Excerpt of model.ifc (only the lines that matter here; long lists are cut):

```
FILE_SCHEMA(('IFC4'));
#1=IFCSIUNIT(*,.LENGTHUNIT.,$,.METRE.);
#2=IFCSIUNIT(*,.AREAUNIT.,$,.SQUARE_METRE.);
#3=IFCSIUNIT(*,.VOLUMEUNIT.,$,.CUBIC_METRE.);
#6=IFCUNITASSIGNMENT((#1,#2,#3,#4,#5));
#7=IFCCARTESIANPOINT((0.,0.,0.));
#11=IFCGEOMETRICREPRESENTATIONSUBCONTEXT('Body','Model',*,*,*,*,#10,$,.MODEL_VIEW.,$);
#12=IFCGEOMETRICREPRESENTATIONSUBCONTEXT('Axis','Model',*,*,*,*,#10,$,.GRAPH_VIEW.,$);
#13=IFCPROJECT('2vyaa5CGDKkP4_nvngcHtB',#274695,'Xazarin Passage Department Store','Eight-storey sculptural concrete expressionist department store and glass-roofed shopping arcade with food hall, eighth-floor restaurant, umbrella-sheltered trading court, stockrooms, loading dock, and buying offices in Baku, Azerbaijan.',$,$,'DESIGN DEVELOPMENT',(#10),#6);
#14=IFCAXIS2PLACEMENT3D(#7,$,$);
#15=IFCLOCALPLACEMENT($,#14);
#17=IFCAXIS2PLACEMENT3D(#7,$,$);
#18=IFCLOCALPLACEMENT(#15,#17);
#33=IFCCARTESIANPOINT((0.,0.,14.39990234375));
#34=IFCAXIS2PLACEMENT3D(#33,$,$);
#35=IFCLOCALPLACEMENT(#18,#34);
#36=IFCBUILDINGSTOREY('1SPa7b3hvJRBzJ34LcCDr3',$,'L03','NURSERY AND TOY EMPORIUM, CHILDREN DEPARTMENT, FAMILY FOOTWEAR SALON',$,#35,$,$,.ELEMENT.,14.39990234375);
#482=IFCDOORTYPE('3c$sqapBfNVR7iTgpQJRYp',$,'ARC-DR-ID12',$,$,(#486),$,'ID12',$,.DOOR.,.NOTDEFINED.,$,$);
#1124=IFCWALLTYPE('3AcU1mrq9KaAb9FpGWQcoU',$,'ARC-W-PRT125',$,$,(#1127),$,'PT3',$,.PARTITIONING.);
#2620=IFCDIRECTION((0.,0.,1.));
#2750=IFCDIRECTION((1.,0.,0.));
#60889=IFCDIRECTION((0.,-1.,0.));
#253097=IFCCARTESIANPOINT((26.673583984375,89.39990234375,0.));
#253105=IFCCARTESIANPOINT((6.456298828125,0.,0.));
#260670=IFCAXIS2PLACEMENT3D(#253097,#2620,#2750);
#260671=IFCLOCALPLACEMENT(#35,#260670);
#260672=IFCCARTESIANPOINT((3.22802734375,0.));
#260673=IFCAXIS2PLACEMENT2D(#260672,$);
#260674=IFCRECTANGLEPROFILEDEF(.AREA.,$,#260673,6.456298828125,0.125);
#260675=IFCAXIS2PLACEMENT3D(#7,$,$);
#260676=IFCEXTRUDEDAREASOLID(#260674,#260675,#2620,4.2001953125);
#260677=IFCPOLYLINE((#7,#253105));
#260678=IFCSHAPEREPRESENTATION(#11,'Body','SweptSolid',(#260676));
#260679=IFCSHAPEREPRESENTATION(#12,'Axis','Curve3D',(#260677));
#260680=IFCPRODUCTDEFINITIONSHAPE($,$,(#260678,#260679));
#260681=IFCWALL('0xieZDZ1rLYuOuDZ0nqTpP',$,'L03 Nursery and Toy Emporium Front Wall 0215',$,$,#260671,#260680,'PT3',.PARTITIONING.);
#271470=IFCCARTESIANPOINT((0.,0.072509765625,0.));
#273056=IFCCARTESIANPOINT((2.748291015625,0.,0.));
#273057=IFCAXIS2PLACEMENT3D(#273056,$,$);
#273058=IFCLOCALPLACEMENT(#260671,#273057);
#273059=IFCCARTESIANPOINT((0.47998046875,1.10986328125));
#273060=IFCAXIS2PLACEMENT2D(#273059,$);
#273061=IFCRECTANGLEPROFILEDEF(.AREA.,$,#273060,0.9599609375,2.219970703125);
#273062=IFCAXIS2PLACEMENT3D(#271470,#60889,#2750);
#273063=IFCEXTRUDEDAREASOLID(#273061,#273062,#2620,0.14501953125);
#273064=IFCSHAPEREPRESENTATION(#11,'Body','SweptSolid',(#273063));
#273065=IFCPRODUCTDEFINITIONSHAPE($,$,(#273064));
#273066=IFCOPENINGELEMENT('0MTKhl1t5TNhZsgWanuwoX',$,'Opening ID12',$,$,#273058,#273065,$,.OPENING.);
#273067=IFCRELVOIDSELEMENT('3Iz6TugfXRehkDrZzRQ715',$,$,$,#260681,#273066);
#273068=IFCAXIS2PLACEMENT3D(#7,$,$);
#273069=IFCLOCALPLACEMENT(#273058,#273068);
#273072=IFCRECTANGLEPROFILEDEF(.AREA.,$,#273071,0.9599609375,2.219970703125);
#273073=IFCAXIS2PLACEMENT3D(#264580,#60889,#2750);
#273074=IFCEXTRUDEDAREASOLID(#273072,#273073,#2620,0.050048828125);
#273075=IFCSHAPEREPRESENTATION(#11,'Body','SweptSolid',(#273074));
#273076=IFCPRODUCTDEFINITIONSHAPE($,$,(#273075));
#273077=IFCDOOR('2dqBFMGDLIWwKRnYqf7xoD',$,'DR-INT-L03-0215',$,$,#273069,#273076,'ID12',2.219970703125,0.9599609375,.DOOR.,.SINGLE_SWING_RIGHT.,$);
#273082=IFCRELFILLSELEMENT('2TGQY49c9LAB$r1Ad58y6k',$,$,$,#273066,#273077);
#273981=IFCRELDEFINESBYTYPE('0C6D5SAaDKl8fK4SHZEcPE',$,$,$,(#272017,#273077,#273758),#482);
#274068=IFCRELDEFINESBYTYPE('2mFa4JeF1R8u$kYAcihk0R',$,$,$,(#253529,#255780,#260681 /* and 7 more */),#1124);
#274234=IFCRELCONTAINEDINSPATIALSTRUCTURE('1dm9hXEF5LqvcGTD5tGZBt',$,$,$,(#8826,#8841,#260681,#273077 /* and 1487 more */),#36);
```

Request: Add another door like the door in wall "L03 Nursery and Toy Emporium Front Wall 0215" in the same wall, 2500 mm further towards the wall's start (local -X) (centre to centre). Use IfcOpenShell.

```python
import ifcopenshell
import ifcopenshell.api.feature
import ifcopenshell.api.geometry
import ifcopenshell.api.root
import ifcopenshell.geom
import ifcopenshell.util.element
import ifcopenshell.util.placement
import ifcopenshell.util.shape
import ifcopenshell.util.unit

model = ifcopenshell.open("model.ifc")
unit_scale = ifcopenshell.util.unit.calculate_unit_scale(model)
settings = ifcopenshell.geom.settings()


def volume(element):
    """Net volume in cubic metres, openings subtracted."""
    shape = ifcopenshell.geom.create_shape(settings, element)
    return ifcopenshell.util.shape.get_volume(shape.geometry)


door = model.by_id(273077)
opening = door.FillsVoids[0].RelatingOpeningElement
wall = opening.VoidsElements[0].RelatingBuildingElement
before = volume(wall)
shift = ifcopenshell.util.placement.get_local_placement(wall.ObjectPlacement)[:3, 0] * -2.5 / unit_scale

# copy_class copies the void relationship, type, container and properties, but no geometry.
new_opening = ifcopenshell.api.root.copy_class(model, product=opening)
new_opening.Representation = ifcopenshell.util.element.copy_deep(
    model, opening.Representation, exclude=["IfcGeometricRepresentationContext", "IfcRepresentationMap"]
)
new_door = ifcopenshell.api.root.copy_class(model, product=door)
new_door.Representation = ifcopenshell.util.element.copy_deep(
    model, door.Representation, exclude=["IfcGeometricRepresentationContext", "IfcRepresentationMap"]
)
new_door.Tag = None
ifcopenshell.api.feature.add_filling(model, opening=new_opening, element=new_door)

for old, new in ((opening, new_opening), (door, new_door)):
    matrix = ifcopenshell.util.placement.get_local_placement(old.ObjectPlacement)
    matrix[:3, 3] += shift
    ifcopenshell.api.geometry.edit_object_placement(model, product=new, matrix=matrix, is_si=False)

after = volume(wall)

print(f"wall volume {before:.3f} -> {after:.3f} m3")

model.write("model_rev.ifc")
```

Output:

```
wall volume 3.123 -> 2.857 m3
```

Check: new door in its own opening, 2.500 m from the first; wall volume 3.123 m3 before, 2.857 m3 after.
